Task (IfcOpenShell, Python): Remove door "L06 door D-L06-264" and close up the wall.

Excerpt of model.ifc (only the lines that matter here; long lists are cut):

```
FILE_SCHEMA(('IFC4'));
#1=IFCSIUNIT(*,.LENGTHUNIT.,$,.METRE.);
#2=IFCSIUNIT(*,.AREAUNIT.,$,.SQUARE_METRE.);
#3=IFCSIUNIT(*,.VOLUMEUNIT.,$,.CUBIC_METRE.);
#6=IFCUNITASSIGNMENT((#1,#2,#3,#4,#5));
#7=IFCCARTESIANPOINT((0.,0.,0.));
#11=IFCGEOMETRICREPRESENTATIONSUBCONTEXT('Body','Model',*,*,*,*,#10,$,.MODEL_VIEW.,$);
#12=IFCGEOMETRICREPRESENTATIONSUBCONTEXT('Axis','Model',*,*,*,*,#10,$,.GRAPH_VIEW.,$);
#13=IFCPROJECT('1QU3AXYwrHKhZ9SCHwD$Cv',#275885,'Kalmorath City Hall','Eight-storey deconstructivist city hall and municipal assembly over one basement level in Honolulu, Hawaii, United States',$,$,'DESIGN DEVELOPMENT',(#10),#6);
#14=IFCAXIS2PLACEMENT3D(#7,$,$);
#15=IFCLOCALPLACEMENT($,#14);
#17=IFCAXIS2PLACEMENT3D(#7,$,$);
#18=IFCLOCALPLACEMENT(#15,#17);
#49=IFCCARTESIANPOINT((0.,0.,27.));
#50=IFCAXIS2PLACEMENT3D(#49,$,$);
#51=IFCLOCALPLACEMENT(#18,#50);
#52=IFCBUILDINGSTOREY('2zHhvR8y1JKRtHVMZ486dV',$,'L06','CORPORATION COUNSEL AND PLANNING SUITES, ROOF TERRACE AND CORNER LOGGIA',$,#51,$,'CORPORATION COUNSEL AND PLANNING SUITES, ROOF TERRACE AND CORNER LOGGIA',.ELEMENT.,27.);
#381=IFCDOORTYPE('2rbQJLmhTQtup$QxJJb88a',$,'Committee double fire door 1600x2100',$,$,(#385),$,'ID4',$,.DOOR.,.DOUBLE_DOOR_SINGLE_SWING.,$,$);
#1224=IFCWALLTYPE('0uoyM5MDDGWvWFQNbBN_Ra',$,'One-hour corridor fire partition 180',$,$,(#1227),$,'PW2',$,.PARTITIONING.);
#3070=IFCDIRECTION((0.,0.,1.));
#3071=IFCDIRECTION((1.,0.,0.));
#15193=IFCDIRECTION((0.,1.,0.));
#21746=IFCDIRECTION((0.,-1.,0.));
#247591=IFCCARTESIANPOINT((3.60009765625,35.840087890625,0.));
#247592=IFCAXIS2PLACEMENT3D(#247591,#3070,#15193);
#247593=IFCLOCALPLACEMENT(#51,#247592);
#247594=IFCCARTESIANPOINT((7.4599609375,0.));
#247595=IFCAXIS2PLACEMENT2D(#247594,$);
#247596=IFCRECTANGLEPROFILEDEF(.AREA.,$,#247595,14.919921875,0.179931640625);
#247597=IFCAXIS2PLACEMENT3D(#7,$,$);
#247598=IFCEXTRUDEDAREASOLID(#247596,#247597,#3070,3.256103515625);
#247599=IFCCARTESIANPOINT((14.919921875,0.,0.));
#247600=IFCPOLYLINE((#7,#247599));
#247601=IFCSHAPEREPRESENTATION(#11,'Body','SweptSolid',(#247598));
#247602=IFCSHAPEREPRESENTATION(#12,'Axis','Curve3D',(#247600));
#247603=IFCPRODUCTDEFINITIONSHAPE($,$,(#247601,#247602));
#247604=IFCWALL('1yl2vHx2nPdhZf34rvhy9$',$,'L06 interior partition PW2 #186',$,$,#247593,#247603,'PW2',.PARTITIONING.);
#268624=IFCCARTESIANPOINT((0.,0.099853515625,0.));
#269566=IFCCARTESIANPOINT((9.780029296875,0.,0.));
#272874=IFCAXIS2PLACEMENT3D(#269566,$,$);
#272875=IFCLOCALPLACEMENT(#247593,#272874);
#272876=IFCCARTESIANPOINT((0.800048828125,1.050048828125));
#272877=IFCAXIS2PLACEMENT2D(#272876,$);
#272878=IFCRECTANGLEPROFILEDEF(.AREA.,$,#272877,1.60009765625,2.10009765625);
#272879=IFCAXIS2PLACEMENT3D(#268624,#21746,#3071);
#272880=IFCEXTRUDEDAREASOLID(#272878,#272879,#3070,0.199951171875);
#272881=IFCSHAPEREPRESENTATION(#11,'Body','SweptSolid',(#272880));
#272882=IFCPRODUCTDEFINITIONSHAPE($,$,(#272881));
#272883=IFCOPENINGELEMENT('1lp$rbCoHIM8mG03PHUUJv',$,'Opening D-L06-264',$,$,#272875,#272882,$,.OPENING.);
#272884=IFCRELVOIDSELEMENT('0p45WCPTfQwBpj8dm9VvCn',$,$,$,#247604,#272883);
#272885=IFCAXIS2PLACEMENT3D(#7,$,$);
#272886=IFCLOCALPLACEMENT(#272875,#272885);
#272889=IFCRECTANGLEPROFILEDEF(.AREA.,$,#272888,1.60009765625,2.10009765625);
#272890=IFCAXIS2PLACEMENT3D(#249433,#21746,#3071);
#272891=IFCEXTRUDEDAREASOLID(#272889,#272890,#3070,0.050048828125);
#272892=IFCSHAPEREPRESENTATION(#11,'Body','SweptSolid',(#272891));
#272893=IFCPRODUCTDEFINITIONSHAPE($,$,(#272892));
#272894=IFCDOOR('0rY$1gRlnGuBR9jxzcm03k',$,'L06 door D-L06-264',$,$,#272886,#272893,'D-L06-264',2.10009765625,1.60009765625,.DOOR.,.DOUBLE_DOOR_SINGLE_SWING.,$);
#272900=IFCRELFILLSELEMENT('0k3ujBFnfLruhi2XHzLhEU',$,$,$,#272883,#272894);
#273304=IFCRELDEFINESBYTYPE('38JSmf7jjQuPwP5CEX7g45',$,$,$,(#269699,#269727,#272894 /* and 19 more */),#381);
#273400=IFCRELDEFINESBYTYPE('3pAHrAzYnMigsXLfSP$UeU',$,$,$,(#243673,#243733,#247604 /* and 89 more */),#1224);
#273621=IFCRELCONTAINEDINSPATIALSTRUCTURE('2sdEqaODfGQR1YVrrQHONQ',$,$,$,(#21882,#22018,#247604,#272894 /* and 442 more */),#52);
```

```python
import ifcopenshell
import ifcopenshell.api.feature
import ifcopenshell.api.root
import ifcopenshell.geom
import ifcopenshell.util.shape

model = ifcopenshell.open("model.ifc")
settings = ifcopenshell.geom.settings()


def volume(element):
    """Net volume in cubic metres, openings subtracted."""
    shape = ifcopenshell.geom.create_shape(settings, element)
    return ifcopenshell.util.shape.get_volume(shape.geometry)


door = model.by_guid("0rY$1gRlnGuBR9jxzcm03k")
opening = door.FillsVoids[0].RelatingOpeningElement
wall = opening.VoidsElements[0].RelatingBuildingElement
before = volume(wall)

ifcopenshell.api.root.remove_product(model, product=door)
ifcopenshell.api.feature.remove_feature(model, feature=opening)

after = volume(wall)

print(f"wall volume {before:.3f} -> {after:.3f} m3")

model.write("model_edited.ifc")
```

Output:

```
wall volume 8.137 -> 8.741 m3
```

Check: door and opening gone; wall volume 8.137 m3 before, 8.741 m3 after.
